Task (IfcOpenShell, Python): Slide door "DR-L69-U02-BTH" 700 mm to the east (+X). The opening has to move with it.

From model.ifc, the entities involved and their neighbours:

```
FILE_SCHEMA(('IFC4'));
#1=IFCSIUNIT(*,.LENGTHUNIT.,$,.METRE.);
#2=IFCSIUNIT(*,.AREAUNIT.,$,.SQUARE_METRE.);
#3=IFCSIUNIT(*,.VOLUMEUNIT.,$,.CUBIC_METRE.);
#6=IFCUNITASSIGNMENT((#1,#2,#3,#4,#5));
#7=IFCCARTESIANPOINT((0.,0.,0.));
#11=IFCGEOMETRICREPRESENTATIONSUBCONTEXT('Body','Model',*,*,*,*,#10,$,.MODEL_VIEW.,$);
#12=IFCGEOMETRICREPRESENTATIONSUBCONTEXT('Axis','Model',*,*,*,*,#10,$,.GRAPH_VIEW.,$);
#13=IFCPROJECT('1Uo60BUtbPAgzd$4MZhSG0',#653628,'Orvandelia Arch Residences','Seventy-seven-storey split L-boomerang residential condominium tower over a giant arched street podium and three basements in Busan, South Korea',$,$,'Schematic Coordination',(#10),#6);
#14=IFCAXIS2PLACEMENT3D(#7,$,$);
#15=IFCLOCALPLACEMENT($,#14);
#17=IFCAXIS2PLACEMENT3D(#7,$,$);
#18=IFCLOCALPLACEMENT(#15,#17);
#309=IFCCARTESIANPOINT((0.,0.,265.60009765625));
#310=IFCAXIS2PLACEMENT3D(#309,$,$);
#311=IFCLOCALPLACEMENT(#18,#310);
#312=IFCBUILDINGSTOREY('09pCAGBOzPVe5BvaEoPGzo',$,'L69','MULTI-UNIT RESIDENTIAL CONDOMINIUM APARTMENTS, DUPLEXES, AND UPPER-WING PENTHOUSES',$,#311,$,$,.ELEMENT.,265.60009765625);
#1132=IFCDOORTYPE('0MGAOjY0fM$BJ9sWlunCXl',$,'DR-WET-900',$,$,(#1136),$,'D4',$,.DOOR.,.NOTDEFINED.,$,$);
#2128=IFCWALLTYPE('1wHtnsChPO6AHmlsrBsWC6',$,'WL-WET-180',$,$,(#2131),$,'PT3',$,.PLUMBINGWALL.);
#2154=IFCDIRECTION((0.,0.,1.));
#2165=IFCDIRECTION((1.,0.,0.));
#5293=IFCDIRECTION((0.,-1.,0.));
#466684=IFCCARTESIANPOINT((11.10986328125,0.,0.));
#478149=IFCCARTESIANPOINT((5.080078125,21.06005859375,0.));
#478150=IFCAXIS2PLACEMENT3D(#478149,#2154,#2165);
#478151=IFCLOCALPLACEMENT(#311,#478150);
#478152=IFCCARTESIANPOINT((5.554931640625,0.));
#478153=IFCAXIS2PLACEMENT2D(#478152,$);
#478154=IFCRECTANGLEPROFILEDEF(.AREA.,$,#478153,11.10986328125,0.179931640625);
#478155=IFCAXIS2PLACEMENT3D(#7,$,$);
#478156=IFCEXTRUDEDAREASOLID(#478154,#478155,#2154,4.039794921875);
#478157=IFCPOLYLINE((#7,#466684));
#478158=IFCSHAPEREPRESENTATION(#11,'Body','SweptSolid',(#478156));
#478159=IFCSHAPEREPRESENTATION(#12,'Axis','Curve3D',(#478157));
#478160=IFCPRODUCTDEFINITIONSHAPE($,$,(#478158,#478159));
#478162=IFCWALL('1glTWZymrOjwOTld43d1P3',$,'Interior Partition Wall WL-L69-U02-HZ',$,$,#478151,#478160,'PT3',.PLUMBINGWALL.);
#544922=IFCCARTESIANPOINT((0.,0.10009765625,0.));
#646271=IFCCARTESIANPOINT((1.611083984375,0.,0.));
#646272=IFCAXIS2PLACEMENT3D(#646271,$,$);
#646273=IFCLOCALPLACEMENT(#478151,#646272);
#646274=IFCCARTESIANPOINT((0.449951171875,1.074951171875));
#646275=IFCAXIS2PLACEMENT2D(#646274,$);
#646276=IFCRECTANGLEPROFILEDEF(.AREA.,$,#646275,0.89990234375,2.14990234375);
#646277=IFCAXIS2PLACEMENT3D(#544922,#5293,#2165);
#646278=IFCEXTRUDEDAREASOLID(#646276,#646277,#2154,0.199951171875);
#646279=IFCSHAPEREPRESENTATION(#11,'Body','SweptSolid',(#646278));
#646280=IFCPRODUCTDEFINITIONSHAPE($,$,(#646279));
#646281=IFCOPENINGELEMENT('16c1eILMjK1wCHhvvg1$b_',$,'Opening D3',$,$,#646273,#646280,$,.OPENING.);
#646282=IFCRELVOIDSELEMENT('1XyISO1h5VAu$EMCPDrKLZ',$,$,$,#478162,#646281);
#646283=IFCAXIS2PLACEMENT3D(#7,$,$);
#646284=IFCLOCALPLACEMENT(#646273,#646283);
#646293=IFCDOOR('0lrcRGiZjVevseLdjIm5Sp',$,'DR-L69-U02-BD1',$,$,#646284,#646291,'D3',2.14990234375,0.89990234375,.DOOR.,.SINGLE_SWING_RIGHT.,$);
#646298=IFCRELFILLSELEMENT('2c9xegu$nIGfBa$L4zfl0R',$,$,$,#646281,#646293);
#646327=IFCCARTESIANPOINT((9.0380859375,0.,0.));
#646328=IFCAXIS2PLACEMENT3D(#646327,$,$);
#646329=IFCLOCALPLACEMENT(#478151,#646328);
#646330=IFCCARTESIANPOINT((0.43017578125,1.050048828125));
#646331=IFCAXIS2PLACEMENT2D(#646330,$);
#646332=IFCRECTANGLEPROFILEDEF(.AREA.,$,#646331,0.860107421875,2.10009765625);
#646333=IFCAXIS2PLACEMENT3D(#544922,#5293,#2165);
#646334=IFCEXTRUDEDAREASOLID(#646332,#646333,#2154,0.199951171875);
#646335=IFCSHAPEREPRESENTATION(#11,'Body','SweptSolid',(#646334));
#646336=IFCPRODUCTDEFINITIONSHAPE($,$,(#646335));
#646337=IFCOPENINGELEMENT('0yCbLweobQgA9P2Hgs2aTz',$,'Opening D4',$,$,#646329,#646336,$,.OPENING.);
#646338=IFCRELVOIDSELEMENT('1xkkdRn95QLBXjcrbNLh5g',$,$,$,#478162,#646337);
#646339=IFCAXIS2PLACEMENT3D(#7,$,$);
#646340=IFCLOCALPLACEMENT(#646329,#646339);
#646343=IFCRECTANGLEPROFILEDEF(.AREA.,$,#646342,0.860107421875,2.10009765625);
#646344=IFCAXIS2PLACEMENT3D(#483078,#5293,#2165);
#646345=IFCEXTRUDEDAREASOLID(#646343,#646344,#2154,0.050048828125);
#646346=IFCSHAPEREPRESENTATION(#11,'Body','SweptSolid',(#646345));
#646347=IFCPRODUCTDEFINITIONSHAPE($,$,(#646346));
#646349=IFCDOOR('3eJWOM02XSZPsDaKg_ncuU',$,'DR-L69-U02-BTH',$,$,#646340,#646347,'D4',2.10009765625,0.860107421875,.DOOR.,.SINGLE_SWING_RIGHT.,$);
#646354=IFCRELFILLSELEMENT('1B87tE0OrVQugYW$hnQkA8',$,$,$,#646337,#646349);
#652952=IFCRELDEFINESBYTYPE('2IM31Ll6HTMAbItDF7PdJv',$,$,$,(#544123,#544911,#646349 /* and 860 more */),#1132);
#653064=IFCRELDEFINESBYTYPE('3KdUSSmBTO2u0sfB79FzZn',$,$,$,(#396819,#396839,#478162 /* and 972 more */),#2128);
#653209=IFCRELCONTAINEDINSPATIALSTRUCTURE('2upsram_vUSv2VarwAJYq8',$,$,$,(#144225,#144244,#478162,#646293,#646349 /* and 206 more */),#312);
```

```python
import ifcopenshell
import ifcopenshell.api.geometry
import ifcopenshell.util.placement

model = ifcopenshell.open("model.ifc")

door = model.by_id(646349)
opening = door.FillsVoids[0].RelatingOpeningElement
wall = opening.VoidsElements[0].RelatingBuildingElement

wall_matrix = ifcopenshell.util.placement.get_local_placement(wall.ObjectPlacement)
shift = wall_matrix[:3, 0] * 0.7
before = ifcopenshell.util.placement.get_local_placement(door.ObjectPlacement)[:3, 3].copy()

# The door is placed relative to its opening, so it follows when the opening moves.
matrix = ifcopenshell.util.placement.get_local_placement(opening.ObjectPlacement)
matrix[:3, 3] += shift
ifcopenshell.api.geometry.edit_object_placement(
    model, product=opening, matrix=matrix, is_si=False, should_transform_children=True
)

after = ifcopenshell.util.placement.get_local_placement(door.ObjectPlacement)[:3, 3]
print("door moved by", (after - before).round(3) + 0.0)

model.write("model_updated.ifc")
```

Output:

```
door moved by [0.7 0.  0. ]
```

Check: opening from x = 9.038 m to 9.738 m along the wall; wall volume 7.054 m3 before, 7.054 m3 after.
